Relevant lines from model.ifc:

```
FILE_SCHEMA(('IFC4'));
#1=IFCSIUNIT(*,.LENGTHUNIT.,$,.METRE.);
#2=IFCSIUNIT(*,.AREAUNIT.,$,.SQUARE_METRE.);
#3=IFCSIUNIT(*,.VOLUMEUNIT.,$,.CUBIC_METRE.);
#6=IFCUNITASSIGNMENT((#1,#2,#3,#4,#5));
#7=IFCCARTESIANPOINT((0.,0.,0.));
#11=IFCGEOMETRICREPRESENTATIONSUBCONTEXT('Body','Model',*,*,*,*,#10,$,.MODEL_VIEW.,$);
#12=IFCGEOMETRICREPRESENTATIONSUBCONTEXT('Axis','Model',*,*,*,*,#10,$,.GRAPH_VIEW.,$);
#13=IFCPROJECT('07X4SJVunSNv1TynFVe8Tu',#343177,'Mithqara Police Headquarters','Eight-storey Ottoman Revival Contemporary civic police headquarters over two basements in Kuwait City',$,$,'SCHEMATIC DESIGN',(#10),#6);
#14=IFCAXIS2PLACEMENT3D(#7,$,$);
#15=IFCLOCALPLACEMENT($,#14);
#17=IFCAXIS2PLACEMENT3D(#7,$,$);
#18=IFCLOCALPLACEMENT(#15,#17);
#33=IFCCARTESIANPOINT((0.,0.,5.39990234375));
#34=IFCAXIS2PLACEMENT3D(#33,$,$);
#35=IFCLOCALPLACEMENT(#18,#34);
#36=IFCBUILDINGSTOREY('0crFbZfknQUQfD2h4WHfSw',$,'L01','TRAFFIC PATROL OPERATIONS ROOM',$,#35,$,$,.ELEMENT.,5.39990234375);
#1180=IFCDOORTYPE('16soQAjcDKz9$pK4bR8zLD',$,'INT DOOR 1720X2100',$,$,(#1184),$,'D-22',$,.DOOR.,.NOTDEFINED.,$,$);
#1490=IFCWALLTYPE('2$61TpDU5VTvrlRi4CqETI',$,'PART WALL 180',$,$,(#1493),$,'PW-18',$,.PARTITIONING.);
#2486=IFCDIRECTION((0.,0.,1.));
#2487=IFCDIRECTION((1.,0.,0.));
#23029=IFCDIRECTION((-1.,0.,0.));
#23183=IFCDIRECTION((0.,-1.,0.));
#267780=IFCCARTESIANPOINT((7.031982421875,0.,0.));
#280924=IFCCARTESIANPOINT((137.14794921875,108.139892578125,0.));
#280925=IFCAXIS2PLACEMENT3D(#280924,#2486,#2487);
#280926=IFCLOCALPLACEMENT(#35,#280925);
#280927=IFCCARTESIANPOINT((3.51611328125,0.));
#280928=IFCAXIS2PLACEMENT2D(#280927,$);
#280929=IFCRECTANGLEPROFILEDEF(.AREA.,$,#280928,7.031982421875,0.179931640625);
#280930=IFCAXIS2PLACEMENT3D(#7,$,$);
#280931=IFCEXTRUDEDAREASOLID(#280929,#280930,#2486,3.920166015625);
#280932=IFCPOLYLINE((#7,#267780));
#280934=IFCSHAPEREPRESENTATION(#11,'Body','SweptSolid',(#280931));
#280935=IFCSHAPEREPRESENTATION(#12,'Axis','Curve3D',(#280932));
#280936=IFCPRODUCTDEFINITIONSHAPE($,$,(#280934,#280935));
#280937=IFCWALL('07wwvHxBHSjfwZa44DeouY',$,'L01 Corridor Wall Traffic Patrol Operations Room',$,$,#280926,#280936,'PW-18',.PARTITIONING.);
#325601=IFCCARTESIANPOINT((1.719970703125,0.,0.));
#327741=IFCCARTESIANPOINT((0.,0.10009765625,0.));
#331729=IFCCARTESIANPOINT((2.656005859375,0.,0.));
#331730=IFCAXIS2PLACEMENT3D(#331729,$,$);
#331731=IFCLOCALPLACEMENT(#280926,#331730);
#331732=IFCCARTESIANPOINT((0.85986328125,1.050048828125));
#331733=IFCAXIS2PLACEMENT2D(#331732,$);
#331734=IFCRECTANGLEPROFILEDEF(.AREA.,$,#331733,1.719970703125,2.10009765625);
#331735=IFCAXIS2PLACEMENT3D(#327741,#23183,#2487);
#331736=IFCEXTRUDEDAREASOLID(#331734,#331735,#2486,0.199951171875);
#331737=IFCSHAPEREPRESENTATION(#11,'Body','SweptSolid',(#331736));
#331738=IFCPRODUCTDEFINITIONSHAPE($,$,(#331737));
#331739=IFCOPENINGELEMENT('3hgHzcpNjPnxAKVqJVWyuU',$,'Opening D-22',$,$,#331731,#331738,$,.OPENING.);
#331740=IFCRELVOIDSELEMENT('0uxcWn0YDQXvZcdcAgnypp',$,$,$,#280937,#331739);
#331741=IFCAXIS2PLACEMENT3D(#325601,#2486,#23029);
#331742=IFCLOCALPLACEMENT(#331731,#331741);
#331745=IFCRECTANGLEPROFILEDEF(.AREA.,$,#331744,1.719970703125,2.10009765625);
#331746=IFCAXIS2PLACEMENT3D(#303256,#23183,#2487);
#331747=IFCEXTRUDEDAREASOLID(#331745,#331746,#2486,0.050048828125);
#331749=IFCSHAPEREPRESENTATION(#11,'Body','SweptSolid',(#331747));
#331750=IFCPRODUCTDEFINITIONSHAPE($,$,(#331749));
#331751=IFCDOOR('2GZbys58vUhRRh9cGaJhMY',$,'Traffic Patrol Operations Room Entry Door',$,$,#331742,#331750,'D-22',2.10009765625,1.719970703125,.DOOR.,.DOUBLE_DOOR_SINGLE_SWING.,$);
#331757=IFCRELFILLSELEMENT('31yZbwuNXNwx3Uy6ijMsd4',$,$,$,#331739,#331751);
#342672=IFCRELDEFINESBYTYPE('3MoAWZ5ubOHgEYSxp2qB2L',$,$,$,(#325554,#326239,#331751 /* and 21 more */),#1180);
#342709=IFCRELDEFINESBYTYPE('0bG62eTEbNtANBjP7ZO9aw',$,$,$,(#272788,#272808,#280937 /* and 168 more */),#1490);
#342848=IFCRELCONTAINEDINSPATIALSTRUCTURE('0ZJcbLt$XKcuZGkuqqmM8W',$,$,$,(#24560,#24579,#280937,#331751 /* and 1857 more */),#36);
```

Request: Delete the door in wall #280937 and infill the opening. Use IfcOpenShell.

```python
import ifcopenshell
import ifcopenshell.api.feature
import ifcopenshell.api.root
import ifcopenshell.geom
import ifcopenshell.util.shape

model = ifcopenshell.open("model.ifc")
settings = ifcopenshell.geom.settings()


def volume(element):
    """Net volume in cubic metres, openings subtracted."""
    shape = ifcopenshell.geom.create_shape(settings, element)
    return ifcopenshell.util.shape.get_volume(shape.geometry)


door = model.by_id(331751)
opening = door.FillsVoids[0].RelatingOpeningElement
wall = opening.VoidsElements[0].RelatingBuildingElement
before = volume(wall)

ifcopenshell.api.root.remove_product(model, product=door)
ifcopenshell.api.feature.remove_feature(model, feature=opening)

after = volume(wall)

print(f"wall volume {before:.3f} -> {after:.3f} m3")

model.write("model_v2.ifc")
```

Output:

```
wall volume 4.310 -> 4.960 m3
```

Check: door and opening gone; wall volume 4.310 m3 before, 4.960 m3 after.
